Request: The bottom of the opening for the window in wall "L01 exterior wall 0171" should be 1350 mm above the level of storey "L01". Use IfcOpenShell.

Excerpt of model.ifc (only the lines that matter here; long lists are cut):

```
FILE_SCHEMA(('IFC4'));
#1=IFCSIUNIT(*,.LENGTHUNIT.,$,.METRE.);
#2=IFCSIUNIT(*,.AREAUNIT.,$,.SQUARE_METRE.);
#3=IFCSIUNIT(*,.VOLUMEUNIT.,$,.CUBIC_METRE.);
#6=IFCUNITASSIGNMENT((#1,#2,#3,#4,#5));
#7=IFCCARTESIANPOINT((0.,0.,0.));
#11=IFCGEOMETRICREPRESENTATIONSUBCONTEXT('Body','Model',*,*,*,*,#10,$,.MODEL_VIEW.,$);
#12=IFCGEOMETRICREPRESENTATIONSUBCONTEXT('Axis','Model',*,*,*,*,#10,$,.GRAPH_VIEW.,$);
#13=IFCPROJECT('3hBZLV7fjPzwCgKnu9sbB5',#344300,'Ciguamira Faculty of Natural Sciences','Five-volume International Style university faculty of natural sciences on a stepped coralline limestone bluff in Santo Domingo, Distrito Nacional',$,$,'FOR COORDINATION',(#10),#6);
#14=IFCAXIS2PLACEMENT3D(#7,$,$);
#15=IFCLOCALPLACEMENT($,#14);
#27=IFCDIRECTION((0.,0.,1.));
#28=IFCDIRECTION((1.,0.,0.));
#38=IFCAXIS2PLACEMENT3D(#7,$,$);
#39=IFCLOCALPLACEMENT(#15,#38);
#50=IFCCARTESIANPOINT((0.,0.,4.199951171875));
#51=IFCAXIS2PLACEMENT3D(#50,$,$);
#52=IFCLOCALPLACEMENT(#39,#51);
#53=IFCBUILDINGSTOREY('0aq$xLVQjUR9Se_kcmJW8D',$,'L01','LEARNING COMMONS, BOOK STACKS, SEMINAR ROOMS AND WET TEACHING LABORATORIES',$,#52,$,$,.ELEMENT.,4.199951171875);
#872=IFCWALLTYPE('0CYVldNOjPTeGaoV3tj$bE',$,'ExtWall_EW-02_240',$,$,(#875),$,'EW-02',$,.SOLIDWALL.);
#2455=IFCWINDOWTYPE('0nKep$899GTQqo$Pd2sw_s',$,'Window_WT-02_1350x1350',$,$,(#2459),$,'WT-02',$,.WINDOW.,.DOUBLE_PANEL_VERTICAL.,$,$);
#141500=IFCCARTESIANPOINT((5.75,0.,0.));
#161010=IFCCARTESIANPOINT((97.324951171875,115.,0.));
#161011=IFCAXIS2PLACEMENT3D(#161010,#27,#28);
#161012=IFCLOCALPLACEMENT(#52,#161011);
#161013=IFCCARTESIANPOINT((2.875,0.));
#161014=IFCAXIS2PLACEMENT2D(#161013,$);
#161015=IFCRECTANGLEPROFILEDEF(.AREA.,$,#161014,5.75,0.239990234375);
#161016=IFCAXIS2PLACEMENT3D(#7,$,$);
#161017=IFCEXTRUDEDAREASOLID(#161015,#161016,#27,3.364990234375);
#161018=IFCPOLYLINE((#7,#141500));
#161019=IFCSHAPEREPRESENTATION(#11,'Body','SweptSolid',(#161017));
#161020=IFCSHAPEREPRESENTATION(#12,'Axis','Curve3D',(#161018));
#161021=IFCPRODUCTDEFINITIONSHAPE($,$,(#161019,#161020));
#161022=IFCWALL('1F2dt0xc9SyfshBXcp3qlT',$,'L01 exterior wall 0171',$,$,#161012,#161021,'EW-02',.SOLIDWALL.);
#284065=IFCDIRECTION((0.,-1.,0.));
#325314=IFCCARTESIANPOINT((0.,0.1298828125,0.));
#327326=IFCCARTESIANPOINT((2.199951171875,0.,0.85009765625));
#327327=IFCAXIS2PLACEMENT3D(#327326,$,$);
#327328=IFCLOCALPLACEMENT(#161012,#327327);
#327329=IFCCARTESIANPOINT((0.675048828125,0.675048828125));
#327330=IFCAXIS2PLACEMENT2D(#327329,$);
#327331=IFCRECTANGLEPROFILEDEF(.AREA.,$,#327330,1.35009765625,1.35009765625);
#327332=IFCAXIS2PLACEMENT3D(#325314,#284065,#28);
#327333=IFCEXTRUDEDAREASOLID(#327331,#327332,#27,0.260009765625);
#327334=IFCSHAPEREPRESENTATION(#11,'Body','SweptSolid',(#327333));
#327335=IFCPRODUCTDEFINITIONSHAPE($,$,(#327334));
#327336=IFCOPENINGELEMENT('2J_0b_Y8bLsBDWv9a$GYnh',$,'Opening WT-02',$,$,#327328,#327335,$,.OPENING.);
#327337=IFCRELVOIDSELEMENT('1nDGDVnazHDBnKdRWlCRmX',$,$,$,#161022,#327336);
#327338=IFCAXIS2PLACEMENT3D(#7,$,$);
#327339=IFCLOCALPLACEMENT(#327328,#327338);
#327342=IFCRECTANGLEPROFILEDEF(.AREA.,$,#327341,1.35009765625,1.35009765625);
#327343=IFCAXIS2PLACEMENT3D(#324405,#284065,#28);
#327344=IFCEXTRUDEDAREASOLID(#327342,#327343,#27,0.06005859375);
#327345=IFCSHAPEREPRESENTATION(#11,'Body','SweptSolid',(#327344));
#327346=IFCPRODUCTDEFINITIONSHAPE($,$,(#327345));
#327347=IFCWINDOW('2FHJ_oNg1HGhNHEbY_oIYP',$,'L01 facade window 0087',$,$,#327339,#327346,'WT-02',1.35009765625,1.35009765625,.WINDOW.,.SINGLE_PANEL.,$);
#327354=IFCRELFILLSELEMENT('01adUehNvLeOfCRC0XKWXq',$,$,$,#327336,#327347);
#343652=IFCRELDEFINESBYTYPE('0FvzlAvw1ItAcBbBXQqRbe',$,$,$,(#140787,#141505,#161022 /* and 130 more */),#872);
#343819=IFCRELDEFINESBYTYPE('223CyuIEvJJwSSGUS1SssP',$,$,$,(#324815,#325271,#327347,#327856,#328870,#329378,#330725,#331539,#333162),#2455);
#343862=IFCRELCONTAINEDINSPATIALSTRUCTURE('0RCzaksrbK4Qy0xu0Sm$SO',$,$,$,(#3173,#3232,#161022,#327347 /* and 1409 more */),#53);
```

```python
import numpy as np
import ifcopenshell
import ifcopenshell.api.geometry
import ifcopenshell.geom
import ifcopenshell.util.element
import ifcopenshell.util.placement
import ifcopenshell.util.shape
import ifcopenshell.util.unit

model = ifcopenshell.open("model.ifc")
unit_scale = ifcopenshell.util.unit.calculate_unit_scale(model)

window = model.by_guid("2FHJ_oNg1HGhNHEbY_oIYP")
opening = window.FillsVoids[0].RelatingOpeningElement
storey = ifcopenshell.util.element.get_container(window, ifc_class="IfcBuildingStorey")
level = ifcopenshell.util.placement.get_local_placement(storey.ObjectPlacement)[2, 3]

# The opening's origin need not be at the sill, so measure its lowest point.
shape = ifcopenshell.geom.create_shape(ifcopenshell.geom.settings(), opening)
bottom = ifcopenshell.util.shape.get_shape_bottom_elevation(shape, shape.geometry) / unit_scale
dz = level + 1.35 / unit_scale - bottom

shift = np.array([0.0, 0.0, dz])
# The window is placed relative to its opening, so it follows when the opening moves.
matrix = ifcopenshell.util.placement.get_local_placement(opening.ObjectPlacement)
matrix[:3, 3] += shift
ifcopenshell.api.geometry.edit_object_placement(
    model, product=opening, matrix=matrix, is_si=False, should_transform_children=True
)

print(f"moved by {dz * unit_scale:+.3f} m")

model.write("model-out.ifc")
```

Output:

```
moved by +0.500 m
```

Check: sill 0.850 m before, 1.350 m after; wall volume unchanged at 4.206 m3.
